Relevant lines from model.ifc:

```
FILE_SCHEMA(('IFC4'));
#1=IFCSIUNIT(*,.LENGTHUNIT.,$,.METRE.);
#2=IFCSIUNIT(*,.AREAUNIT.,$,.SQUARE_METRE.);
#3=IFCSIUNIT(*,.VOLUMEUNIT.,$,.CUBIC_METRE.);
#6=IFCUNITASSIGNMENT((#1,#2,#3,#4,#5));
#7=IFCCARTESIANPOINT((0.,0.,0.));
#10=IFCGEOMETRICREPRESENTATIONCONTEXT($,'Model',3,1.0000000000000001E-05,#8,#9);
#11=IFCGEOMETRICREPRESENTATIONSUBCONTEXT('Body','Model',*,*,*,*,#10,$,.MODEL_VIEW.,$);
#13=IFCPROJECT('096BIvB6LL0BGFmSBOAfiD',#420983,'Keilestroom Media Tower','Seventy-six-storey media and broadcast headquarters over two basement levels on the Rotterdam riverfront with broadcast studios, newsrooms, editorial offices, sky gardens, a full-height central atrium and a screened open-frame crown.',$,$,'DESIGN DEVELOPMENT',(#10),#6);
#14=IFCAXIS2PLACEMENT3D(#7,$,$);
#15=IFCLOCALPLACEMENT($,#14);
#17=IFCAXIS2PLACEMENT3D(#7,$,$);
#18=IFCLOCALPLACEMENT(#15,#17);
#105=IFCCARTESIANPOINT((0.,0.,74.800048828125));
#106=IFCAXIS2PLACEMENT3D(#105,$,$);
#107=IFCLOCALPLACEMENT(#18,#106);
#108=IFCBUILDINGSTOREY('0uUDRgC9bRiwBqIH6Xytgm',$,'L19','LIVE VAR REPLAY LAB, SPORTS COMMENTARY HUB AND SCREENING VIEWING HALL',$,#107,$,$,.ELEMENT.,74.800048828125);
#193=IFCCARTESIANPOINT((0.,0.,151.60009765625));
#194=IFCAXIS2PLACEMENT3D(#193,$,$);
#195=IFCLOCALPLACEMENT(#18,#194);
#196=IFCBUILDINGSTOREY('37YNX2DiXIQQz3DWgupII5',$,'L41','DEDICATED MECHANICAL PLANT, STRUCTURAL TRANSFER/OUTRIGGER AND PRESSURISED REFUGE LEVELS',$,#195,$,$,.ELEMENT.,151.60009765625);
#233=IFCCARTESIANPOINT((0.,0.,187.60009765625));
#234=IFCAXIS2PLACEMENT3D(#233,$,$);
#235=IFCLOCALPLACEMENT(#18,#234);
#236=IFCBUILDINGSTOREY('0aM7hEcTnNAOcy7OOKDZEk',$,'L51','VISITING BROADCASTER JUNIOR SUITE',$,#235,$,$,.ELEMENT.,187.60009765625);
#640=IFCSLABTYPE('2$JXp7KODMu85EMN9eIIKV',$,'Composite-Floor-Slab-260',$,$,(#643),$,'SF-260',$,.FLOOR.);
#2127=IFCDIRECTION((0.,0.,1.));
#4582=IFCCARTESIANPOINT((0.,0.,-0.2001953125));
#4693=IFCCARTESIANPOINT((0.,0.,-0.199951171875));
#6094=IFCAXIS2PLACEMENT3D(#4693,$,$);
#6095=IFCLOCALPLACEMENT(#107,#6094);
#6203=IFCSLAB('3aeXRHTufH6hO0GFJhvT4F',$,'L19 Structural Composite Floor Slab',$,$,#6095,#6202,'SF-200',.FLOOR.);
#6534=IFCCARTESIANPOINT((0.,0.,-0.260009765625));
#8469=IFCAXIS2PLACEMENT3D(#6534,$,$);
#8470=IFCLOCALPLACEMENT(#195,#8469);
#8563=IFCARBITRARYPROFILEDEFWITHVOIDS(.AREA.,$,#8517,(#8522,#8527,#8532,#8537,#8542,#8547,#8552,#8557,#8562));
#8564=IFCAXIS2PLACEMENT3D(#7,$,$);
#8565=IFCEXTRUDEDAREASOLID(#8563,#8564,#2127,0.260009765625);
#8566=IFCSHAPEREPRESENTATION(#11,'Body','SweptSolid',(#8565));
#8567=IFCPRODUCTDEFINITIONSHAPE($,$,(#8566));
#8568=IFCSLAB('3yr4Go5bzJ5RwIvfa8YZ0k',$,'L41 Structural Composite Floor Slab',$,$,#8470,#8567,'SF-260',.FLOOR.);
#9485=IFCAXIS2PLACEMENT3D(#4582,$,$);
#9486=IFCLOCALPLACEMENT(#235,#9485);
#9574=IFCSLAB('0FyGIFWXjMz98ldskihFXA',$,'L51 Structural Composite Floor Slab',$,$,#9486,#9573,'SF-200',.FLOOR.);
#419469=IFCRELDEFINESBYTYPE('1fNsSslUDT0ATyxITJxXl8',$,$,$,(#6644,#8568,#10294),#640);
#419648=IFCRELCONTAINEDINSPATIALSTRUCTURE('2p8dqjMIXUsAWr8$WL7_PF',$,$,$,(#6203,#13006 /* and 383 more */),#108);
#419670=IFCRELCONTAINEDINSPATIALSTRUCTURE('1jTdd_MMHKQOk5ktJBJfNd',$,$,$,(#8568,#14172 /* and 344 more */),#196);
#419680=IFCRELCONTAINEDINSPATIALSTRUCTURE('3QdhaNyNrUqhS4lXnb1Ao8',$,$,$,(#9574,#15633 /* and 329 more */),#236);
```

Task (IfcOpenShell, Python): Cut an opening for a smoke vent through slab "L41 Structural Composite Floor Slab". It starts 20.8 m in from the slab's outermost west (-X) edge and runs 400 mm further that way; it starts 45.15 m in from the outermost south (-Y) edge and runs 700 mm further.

```python
import numpy as np
import ifcopenshell
import ifcopenshell.api.feature
import ifcopenshell.api.geometry
import ifcopenshell.api.root
import ifcopenshell.geom
import ifcopenshell.util.placement
import ifcopenshell.util.representation
import ifcopenshell.util.shape
import ifcopenshell.util.unit

model = ifcopenshell.open("model.ifc")
unit_scale = ifcopenshell.util.unit.calculate_unit_scale(model)
settings = ifcopenshell.geom.settings()


def volume(element):
    """Net volume in cubic metres, openings subtracted."""
    shape = ifcopenshell.geom.create_shape(settings, element)
    return ifcopenshell.util.shape.get_volume(shape.geometry)


slab = model.by_id(8568)
before = volume(slab)

# Extent in the slab's own axes, in metres. The edges named are its -X and -Y sides.
slab_shape = ifcopenshell.geom.create_shape(settings, slab)
vertices = ifcopenshell.util.shape.get_vertices(slab_shape.geometry)
x_min, y_min, bottom = vertices.min(axis=0)
top = vertices[:, 2].max()

opening = ifcopenshell.api.root.create_entity(model, ifc_class="IfcOpeningElement", name="Smoke vent opening", predefined_type="OPENING")
context = ifcopenshell.util.representation.get_context(model, "Model", "Body", "MODEL_VIEW")
width, depth = 0.4, 0.7
outline = [(0.0, 0.0), (width, 0.0), (width, depth), (0.0, depth), (0.0, 0.0)]
# Overshoot both faces by 50 mm so the cut is clean.
shape = ifcopenshell.api.geometry.add_slab_representation(
    model, context=context, depth=top - bottom + 0.1, polyline=outline
)
ifcopenshell.api.geometry.assign_representation(model, product=opening, representation=shape)

matrix = ifcopenshell.util.placement.get_local_placement(slab.ObjectPlacement)
matrix[:, 3] = matrix @ np.append(np.array([x_min + 20.8, y_min + 45.15, bottom - 0.05]) / unit_scale, 1.0)
ifcopenshell.api.geometry.edit_object_placement(model, product=opening, matrix=matrix, is_si=False)
ifcopenshell.api.feature.add_feature(model, feature=opening, element=slab)

after = volume(slab)

print(f"slab volume {before:.3f} -> {after:.3f} m3")

model.write("model_v2.ifc")
```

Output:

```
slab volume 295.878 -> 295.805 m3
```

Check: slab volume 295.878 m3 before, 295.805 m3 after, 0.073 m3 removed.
